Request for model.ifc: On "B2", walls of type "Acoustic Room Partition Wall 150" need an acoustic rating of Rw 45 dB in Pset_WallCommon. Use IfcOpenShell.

First a look at what the model holds.

```python
import ifcopenshell
import ifcopenshell.util.element

model = ifcopenshell.open("model.ifc")
print(model.schema)
storey = next(s for s in model.by_type("IfcBuildingStorey") if s.Name == "B2")
walls = [e for e in ifcopenshell.util.element.get_decomposition(storey) if e.is_a("IfcWall")]
seen = {}
for e in walls:
    element_type = ifcopenshell.util.element.get_type(e)
    key = (element_type.Name if element_type != e and element_type else None, ifcopenshell.util.element.get_pset(e, "Pset_WallCommon", "AcousticRating"))
    seen[key] = seen.get(key, 0) + 1
for (name, value), count in sorted(seen.items(), key=str):
    print(count, "x", name, "|", value)
```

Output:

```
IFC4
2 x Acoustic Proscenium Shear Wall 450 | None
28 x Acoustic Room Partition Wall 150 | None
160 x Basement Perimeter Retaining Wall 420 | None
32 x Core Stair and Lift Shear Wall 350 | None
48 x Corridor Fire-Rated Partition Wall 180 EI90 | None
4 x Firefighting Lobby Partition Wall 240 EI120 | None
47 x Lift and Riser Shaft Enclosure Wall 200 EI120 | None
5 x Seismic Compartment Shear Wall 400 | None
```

```python
import ifcopenshell
import ifcopenshell.api.pset
import ifcopenshell.util.element

model = ifcopenshell.open("model.ifc")

storey = next(s for s in model.by_type("IfcBuildingStorey") if s.Name == "B2")
walls = [e for e in ifcopenshell.util.element.get_decomposition(storey) if e.is_a("IfcWall")]

count = 0
for e in walls:
    element_type = ifcopenshell.util.element.get_type(e)
    if element_type in (None, e) or element_type.Name != "Acoustic Room Partition Wall 150":
        continue
    # add_pset returns the element's existing set when there is one.
    pset = ifcopenshell.api.pset.add_pset(model, product=e, name="Pset_WallCommon")
    ifcopenshell.api.pset.edit_pset(model, pset=pset, properties={"AcousticRating": "Rw 45 dB"})
    count += 1

print(count, "walls updated")

model.write("model_rev.ifc")
```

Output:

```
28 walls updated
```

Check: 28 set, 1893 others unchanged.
